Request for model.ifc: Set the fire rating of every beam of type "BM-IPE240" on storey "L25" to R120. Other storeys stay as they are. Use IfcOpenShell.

First a look at what the model holds.

```python
import ifcopenshell
import ifcopenshell.util.element

model = ifcopenshell.open("model.ifc")
print(model.schema)
storey = next(s for s in model.by_type("IfcBuildingStorey") if s.Name == "L25")
beams = [e for e in ifcopenshell.util.element.get_decomposition(storey) if e.is_a("IfcBeam")]
seen = {}
for e in beams:
    element_type = ifcopenshell.util.element.get_type(e)
    key = (element_type.Name if element_type != e and element_type else None, ifcopenshell.util.element.get_pset(e, "Pset_BeamCommon", "FireRating"))
    seen[key] = seen.get(key, 0) + 1
for (name, value), count in sorted(seen.items(), key=str):
    print(count, "x", name, "|", value)
```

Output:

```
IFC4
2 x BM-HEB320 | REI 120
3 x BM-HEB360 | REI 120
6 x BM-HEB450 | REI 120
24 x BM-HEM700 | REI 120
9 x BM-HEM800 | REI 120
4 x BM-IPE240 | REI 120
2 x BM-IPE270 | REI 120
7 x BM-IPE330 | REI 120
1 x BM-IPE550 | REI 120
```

```python
import ifcopenshell
import ifcopenshell.api.pset
import ifcopenshell.util.element

model = ifcopenshell.open("model.ifc")

storey = next(s for s in model.by_type("IfcBuildingStorey") if s.Name == "L25")
beams = [e for e in ifcopenshell.util.element.get_decomposition(storey) if e.is_a("IfcBeam")]

count = 0
for e in beams:
    element_type = ifcopenshell.util.element.get_type(e)
    if element_type in (None, e) or element_type.Name != "BM-IPE240":
        continue
    found = ifcopenshell.util.element.get_pset(e, "Pset_BeamCommon", should_inherit=False)
    if found:
        pset = model.by_id(found["id"])
        if len(ifcopenshell.util.element.get_elements_by_pset(pset)) > 1:
            pset = ifcopenshell.api.pset.unshare_pset(model, products=[e], pset=pset)[0]
    else:
        pset = ifcopenshell.api.pset.add_pset(model, product=e, name="Pset_BeamCommon")
    ifcopenshell.api.pset.edit_pset(model, pset=pset, properties={"FireRating": "R120"})
    count += 1

print(count, "beams updated")

model.write("model_updated.ifc")
```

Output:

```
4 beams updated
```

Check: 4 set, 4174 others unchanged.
